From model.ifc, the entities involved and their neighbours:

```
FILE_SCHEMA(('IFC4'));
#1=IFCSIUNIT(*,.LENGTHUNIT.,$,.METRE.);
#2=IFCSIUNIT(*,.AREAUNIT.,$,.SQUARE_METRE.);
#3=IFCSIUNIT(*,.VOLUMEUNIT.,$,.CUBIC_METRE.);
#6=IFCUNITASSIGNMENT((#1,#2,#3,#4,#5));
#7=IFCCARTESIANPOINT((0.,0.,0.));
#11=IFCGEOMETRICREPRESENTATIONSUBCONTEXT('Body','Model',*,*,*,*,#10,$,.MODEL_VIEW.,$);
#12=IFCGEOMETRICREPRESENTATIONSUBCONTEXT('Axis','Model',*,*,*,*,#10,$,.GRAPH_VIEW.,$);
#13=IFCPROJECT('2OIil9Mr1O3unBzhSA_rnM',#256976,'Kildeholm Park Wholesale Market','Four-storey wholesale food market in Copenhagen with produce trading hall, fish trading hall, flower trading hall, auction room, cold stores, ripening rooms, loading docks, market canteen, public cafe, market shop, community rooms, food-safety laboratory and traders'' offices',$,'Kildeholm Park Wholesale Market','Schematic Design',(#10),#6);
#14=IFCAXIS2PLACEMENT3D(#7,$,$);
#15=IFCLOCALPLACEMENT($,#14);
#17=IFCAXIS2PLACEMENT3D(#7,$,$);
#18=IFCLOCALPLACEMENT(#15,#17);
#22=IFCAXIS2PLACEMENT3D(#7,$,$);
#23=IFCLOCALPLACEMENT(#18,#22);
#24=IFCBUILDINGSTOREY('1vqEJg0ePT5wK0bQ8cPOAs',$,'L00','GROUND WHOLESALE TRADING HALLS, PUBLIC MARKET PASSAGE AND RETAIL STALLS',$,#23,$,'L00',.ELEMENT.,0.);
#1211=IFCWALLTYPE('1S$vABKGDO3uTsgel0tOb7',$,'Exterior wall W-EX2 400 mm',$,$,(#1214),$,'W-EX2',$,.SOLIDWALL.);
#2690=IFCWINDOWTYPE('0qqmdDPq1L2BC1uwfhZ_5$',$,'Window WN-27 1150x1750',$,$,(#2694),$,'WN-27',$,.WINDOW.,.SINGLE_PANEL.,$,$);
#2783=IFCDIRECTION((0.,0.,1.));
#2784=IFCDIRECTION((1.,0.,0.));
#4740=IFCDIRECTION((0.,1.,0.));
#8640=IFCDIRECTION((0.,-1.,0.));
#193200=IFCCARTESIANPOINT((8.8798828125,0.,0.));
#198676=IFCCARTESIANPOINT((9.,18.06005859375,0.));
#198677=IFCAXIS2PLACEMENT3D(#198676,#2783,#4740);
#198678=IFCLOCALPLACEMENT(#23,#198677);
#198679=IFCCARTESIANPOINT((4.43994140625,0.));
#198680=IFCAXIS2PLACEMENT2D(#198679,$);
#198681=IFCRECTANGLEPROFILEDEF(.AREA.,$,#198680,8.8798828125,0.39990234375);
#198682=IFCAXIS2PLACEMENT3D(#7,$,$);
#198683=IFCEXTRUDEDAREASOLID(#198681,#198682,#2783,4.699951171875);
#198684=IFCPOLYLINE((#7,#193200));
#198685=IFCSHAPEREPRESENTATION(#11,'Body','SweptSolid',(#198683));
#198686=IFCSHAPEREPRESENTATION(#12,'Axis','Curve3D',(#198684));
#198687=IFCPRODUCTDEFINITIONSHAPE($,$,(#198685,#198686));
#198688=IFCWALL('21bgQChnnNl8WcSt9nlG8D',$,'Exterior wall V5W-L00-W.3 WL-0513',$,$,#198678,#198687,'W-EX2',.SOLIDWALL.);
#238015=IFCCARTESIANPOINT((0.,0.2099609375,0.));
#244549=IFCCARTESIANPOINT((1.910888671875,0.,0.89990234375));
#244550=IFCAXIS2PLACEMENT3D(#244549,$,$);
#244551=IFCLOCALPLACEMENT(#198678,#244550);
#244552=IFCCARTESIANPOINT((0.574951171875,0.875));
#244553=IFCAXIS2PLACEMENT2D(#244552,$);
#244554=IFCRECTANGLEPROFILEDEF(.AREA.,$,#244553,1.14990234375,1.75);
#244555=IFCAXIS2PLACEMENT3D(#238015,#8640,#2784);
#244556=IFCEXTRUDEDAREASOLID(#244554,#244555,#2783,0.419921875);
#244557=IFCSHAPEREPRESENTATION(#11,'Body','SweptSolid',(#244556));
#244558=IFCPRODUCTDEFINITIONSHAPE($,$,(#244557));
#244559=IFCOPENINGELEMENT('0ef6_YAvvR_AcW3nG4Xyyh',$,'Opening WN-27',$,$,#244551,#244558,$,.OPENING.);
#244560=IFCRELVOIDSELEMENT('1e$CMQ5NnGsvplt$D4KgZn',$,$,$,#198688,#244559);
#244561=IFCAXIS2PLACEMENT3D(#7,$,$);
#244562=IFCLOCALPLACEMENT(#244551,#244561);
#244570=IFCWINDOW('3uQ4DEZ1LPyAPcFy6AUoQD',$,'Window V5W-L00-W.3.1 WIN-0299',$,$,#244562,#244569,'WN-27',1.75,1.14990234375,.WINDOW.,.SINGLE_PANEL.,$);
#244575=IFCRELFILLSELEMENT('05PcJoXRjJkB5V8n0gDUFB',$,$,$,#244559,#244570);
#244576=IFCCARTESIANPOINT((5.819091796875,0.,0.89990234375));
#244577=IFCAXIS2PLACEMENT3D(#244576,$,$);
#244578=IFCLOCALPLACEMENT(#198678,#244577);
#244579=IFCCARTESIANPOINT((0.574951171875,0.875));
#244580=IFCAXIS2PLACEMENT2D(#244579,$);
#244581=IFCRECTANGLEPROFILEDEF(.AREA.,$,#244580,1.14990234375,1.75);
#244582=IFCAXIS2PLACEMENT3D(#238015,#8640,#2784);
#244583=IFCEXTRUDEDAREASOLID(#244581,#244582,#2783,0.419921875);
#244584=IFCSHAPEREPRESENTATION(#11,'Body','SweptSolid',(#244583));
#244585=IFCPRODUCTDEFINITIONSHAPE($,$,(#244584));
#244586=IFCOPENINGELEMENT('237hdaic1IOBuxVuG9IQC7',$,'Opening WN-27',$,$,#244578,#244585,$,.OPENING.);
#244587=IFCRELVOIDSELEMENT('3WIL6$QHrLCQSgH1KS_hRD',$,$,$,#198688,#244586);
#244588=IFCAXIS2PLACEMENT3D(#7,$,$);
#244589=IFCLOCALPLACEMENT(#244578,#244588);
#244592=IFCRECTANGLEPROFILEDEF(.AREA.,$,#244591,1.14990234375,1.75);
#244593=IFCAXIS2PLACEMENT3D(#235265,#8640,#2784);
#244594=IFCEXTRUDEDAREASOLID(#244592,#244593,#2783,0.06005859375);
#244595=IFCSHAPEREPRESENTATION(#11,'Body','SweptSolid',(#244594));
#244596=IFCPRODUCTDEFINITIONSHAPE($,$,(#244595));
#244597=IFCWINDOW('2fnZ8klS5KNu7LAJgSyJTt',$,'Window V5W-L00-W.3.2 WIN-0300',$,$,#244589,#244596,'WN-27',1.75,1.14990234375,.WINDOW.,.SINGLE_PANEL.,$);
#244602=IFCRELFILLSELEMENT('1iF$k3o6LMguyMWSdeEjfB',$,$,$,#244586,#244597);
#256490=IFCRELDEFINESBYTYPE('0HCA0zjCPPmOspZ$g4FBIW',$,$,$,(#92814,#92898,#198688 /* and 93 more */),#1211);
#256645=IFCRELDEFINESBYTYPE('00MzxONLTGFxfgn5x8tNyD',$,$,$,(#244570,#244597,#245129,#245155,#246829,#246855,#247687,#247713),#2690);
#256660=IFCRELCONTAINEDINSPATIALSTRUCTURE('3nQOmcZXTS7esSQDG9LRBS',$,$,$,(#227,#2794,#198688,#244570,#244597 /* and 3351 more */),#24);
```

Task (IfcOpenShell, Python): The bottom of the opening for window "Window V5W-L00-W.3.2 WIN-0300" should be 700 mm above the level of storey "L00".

```python
import numpy as np
import ifcopenshell
import ifcopenshell.api.geometry
import ifcopenshell.geom
import ifcopenshell.util.element
import ifcopenshell.util.placement
import ifcopenshell.util.shape
import ifcopenshell.util.unit

model = ifcopenshell.open("model.ifc")
unit_scale = ifcopenshell.util.unit.calculate_unit_scale(model)

window = model.by_id(244597)
opening = window.FillsVoids[0].RelatingOpeningElement
storey = ifcopenshell.util.element.get_container(window, ifc_class="IfcBuildingStorey")
level = ifcopenshell.util.placement.get_local_placement(storey.ObjectPlacement)[2, 3]

# The opening's origin need not be at the sill, so measure its lowest point.
shape = ifcopenshell.geom.create_shape(ifcopenshell.geom.settings(), opening)
bottom = ifcopenshell.util.shape.get_shape_bottom_elevation(shape, shape.geometry) / unit_scale
dz = level + 0.7 / unit_scale - bottom

shift = np.array([0.0, 0.0, dz])
# The window is placed relative to its opening, so it follows when the opening moves.
matrix = ifcopenshell.util.placement.get_local_placement(opening.ObjectPlacement)
matrix[:3, 3] += shift
ifcopenshell.api.geometry.edit_object_placement(
    model, product=opening, matrix=matrix, is_si=False, should_transform_children=True
)

print(f"moved by {dz * unit_scale:+.3f} m")

model.write("model_rev.ifc")
```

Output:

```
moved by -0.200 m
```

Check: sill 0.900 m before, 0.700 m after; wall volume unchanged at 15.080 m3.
